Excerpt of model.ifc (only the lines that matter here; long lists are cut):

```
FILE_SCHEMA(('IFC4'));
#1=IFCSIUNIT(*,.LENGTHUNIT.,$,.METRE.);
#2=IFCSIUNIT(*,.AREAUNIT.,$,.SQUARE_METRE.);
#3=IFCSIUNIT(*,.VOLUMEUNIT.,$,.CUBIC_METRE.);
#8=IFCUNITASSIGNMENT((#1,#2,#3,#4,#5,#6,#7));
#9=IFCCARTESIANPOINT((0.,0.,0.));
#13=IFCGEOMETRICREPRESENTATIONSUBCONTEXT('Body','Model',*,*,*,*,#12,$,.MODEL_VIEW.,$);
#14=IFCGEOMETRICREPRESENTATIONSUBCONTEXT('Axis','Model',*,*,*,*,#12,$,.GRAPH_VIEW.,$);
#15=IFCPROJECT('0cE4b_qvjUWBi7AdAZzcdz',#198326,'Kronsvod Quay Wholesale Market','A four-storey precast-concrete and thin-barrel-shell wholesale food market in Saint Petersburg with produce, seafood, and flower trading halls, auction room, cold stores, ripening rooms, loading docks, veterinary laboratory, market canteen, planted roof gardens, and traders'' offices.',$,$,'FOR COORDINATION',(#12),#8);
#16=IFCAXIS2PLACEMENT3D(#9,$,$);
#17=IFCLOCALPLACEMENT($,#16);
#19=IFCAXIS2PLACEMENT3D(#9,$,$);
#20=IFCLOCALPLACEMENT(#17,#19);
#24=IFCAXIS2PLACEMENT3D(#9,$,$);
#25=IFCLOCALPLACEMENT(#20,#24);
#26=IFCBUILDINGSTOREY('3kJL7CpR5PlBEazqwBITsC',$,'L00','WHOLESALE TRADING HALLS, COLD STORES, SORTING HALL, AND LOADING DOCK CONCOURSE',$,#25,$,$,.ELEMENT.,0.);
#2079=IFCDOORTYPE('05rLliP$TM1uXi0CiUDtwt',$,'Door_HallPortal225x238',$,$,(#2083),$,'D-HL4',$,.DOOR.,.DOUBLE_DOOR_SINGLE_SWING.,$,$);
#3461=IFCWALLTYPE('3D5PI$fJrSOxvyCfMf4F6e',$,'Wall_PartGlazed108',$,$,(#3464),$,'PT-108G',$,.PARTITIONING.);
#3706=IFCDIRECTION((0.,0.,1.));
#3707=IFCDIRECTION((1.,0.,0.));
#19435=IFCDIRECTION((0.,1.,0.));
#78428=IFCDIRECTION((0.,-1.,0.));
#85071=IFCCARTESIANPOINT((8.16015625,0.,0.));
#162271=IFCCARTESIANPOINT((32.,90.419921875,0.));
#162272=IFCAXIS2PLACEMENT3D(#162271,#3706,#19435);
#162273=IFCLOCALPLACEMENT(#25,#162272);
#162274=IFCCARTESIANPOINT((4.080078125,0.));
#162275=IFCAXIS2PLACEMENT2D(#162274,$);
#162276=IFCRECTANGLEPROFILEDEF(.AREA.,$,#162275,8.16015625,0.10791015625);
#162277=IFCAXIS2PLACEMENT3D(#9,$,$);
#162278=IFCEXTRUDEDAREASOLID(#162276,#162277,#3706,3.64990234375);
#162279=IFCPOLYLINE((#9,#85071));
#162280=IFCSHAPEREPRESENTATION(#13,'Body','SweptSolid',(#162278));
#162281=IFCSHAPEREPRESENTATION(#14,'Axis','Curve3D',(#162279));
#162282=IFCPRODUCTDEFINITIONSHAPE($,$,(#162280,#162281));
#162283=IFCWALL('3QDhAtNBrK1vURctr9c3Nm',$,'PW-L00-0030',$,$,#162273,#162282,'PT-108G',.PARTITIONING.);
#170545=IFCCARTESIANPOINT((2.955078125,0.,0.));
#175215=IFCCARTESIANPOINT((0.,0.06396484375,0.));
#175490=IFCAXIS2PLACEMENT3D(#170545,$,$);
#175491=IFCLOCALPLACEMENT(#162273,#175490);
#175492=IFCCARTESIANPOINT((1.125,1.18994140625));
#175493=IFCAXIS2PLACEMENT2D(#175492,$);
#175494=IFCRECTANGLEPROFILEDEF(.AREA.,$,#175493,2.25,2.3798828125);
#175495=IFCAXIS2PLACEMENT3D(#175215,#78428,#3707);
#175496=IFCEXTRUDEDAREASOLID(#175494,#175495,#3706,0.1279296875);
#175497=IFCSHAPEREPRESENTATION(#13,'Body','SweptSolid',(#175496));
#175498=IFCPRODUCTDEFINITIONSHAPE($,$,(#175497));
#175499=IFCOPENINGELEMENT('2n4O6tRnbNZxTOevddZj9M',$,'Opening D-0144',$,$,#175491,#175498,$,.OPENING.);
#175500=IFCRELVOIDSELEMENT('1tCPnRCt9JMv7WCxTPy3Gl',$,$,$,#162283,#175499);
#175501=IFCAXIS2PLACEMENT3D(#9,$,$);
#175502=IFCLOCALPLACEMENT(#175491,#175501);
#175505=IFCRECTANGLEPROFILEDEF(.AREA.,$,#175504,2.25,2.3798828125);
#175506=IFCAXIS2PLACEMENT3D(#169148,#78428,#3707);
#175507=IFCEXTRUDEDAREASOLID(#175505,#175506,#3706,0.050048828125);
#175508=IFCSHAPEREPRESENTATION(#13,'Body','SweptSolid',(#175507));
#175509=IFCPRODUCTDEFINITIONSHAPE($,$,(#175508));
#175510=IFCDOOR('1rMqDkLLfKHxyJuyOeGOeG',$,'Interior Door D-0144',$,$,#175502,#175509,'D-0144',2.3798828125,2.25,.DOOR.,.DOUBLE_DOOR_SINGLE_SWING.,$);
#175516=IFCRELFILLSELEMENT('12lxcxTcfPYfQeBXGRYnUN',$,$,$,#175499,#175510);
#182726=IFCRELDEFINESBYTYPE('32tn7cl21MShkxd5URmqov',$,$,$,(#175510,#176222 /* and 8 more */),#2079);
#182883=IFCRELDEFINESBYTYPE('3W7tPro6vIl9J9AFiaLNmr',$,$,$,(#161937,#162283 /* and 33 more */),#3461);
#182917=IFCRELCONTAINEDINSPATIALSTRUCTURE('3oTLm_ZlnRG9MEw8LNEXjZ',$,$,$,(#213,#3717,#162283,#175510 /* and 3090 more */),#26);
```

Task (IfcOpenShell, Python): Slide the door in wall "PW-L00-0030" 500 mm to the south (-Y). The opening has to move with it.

```python
import ifcopenshell
import ifcopenshell.api.geometry
import ifcopenshell.util.placement
import ifcopenshell.util.unit

model = ifcopenshell.open("model.ifc")
unit_scale = ifcopenshell.util.unit.calculate_unit_scale(model)

door = model.by_id(175510)
opening = door.FillsVoids[0].RelatingOpeningElement
wall = opening.VoidsElements[0].RelatingBuildingElement

wall_matrix = ifcopenshell.util.placement.get_local_placement(wall.ObjectPlacement)
shift = wall_matrix[:3, 0] * -0.5 / unit_scale
before = ifcopenshell.util.placement.get_local_placement(door.ObjectPlacement)[:3, 3].copy()

# The door is placed relative to its opening, so it follows when the opening moves.
matrix = ifcopenshell.util.placement.get_local_placement(opening.ObjectPlacement)
matrix[:3, 3] += shift
ifcopenshell.api.geometry.edit_object_placement(
    model, product=opening, matrix=matrix, is_si=False, should_transform_children=True
)

after = ifcopenshell.util.placement.get_local_placement(door.ObjectPlacement)[:3, 3]
print("door moved by", (after - before).round(3) + 0.0)

model.write("model_rev.ifc")
```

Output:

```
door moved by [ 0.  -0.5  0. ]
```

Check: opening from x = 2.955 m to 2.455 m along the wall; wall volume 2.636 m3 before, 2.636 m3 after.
